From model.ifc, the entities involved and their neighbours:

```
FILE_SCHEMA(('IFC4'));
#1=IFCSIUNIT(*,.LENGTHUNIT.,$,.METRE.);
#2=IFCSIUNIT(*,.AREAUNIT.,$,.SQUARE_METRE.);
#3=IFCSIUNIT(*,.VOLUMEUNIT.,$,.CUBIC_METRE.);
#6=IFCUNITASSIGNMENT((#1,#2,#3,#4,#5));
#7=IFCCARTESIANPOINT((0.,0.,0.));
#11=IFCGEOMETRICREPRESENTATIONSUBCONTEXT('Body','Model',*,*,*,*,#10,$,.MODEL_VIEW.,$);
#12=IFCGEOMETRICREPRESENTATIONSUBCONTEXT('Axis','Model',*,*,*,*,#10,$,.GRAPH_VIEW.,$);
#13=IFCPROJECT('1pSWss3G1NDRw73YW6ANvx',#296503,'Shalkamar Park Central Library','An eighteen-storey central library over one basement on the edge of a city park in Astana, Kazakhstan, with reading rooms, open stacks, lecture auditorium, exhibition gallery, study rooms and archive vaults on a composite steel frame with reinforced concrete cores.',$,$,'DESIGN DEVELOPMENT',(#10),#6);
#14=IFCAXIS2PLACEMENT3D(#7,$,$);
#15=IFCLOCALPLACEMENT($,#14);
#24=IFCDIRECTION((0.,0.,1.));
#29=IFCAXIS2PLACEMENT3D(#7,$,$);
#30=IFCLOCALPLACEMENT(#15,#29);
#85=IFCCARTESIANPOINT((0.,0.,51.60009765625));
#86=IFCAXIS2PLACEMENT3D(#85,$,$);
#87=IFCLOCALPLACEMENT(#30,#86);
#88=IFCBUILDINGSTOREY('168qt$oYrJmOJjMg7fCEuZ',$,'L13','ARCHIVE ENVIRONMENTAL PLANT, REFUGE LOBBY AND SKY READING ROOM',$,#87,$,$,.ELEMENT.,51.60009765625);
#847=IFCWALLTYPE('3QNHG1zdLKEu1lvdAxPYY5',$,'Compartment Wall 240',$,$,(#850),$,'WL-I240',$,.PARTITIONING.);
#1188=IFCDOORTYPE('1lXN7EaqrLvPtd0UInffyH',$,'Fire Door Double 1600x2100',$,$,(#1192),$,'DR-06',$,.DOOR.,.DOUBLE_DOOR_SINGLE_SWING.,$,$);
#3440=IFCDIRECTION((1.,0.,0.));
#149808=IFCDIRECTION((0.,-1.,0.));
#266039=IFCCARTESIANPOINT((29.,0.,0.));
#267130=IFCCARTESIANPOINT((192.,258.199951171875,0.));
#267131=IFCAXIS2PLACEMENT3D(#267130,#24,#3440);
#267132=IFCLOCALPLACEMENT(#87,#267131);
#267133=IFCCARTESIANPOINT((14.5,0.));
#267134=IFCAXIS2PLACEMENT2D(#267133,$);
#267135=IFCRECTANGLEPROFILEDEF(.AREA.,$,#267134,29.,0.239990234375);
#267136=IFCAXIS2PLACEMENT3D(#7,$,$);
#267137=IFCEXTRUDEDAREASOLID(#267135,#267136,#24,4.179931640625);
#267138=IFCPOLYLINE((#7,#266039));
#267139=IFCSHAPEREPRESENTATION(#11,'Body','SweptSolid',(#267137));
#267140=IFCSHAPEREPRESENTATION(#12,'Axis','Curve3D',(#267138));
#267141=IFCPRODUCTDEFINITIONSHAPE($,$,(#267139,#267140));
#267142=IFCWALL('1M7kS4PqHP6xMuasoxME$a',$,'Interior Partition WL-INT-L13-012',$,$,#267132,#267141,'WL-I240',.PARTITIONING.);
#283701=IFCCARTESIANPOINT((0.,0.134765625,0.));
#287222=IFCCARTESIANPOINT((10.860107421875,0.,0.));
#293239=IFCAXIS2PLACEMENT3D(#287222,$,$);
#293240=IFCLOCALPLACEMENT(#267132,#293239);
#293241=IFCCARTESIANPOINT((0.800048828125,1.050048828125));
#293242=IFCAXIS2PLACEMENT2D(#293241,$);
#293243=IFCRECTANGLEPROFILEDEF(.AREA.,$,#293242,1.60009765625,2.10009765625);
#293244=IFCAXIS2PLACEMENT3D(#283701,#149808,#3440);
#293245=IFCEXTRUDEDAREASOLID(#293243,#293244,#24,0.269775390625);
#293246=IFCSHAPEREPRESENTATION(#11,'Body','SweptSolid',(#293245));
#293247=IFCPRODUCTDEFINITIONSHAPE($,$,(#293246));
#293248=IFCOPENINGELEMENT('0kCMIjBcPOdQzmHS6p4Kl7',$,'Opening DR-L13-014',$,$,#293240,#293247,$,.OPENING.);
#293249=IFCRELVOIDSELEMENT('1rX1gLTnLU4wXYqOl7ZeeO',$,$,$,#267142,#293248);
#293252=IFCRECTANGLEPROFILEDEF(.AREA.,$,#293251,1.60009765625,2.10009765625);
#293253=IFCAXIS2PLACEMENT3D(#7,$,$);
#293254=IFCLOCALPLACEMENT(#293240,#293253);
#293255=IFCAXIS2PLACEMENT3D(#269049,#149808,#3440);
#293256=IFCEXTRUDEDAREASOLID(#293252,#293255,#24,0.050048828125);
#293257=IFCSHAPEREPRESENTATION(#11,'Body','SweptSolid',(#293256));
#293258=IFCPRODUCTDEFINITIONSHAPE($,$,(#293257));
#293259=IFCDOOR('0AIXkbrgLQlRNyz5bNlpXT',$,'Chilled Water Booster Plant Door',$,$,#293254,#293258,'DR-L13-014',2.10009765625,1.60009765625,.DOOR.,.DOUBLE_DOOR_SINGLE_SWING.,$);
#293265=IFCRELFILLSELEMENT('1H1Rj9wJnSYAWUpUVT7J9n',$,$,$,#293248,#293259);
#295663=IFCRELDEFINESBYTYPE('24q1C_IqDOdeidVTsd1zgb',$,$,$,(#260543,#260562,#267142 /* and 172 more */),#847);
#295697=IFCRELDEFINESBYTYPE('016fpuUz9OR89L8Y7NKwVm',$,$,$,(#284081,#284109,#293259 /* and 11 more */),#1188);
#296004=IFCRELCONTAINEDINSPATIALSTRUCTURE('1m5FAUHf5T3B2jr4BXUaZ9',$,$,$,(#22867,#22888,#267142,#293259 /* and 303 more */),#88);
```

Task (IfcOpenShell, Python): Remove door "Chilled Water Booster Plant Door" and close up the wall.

```python
import ifcopenshell
import ifcopenshell.api.feature
import ifcopenshell.api.root
import ifcopenshell.geom
import ifcopenshell.util.shape

model = ifcopenshell.open("model.ifc")
settings = ifcopenshell.geom.settings()


def volume(element):
    """Net volume in cubic metres, openings subtracted."""
    shape = ifcopenshell.geom.create_shape(settings, element)
    return ifcopenshell.util.shape.get_volume(shape.geometry)


door = model.by_id(293259)
opening = door.FillsVoids[0].RelatingOpeningElement
wall = opening.VoidsElements[0].RelatingBuildingElement
before = volume(wall)

ifcopenshell.api.root.remove_product(model, product=door)
ifcopenshell.api.feature.remove_feature(model, feature=opening)

after = volume(wall)

print(f"wall volume {before:.3f} -> {after:.3f} m3")

model.write("model_v2.ifc")
```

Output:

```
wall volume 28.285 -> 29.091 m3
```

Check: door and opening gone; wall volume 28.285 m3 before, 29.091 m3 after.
